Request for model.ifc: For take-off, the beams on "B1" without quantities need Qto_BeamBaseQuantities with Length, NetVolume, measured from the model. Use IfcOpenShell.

First a look at what the model holds.

```python
import ifcopenshell
import ifcopenshell.util.element
import ifcopenshell.util.unit

model = ifcopenshell.open("model.ifc")
print(model.schema)
for unit_type in ("LENGTHUNIT", "AREAUNIT", "VOLUMEUNIT"):
    print(unit_type, ifcopenshell.util.unit.calculate_unit_scale(model, unit_type))
storey = next(s for s in model.by_type("IfcBuildingStorey") if s.Name == "B1")
beams = [e for e in ifcopenshell.util.element.get_decomposition(storey) if e.is_a("IfcBeam")]
for e in sorted(beams, key=lambda e: e.id()):
    print(e.id(), e.is_a(), e.Name, list(ifcopenshell.util.element.get_psets(e, qtos_only=True)), sep=" | ")
```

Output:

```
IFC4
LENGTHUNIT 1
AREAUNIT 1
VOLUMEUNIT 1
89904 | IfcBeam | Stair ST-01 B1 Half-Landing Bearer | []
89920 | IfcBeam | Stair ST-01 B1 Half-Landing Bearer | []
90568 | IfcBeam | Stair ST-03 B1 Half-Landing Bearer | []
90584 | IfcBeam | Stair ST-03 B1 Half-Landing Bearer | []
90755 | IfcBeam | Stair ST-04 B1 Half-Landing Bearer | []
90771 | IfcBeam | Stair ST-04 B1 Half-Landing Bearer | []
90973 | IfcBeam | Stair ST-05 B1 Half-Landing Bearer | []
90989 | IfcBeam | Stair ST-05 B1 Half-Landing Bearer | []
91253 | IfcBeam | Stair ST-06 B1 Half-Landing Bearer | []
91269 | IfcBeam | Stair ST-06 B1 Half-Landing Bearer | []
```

```python
import ifcopenshell
import ifcopenshell.api.pset
import ifcopenshell.geom
import ifcopenshell.util.element
import ifcopenshell.util.shape
import ifcopenshell.util.unit

model = ifcopenshell.open("model.ifc")
unit_scale = ifcopenshell.util.unit.calculate_unit_scale(model)
volume_scale = ifcopenshell.util.unit.calculate_unit_scale(model, "VOLUMEUNIT")
settings = ifcopenshell.geom.settings()

storey = next(s for s in model.by_type("IfcBuildingStorey") if s.Name == "B1")
beams = [e for e in ifcopenshell.util.element.get_decomposition(storey) if e.is_a("IfcBeam")]

for e in sorted(beams, key=lambda e: e.id()):
    if ifcopenshell.util.element.get_psets(e, qtos_only=True, should_inherit=False):
        continue
    # Geometry comes back in metres, in the element's own axes.
    shape = ifcopenshell.geom.create_shape(settings, e)
    values = {
        "Length": ifcopenshell.util.shape.get_max_xyz(shape.geometry) / unit_scale,
        "NetVolume": ifcopenshell.util.shape.get_volume(shape.geometry) / volume_scale,
    }
    qto = ifcopenshell.api.pset.add_qto(model, product=e, name="Qto_BeamBaseQuantities")
    ifcopenshell.api.pset.edit_qto(model, qto=qto, properties=values)
    print(e.id(), {k: round(v, 3) for k, v in values.items()})

model.write("model_rev.ifc")
```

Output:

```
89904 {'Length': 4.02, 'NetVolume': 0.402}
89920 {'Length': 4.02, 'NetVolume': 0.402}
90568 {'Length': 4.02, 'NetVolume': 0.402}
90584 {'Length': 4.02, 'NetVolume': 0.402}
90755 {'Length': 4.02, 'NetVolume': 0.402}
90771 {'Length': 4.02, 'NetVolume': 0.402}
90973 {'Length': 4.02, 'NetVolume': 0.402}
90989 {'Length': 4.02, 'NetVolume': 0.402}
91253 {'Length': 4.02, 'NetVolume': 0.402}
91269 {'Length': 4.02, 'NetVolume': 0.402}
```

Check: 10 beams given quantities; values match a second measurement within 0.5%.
